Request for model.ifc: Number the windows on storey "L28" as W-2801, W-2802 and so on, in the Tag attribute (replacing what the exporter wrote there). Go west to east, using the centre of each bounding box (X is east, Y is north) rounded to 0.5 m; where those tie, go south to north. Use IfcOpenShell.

First a look at what the model holds.

```python
import ifcopenshell
import ifcopenshell.util.element
import ifcopenshell.util.placement

model = ifcopenshell.open("model.ifc")
print(model.schema)
storey = next(s for s in model.by_type("IfcBuildingStorey") if s.Name == "L28")
windows = [e for e in ifcopenshell.util.element.get_decomposition(storey) if e.is_a("IfcWindow")]
for e in sorted(windows, key=lambda e: e.id()):
    origin = ifcopenshell.util.placement.get_local_placement(e.ObjectPlacement)[:3, 3]
    print(e.id(), e.Tag, e.Name, origin.round(2) + 0.0, sep=" | ")
```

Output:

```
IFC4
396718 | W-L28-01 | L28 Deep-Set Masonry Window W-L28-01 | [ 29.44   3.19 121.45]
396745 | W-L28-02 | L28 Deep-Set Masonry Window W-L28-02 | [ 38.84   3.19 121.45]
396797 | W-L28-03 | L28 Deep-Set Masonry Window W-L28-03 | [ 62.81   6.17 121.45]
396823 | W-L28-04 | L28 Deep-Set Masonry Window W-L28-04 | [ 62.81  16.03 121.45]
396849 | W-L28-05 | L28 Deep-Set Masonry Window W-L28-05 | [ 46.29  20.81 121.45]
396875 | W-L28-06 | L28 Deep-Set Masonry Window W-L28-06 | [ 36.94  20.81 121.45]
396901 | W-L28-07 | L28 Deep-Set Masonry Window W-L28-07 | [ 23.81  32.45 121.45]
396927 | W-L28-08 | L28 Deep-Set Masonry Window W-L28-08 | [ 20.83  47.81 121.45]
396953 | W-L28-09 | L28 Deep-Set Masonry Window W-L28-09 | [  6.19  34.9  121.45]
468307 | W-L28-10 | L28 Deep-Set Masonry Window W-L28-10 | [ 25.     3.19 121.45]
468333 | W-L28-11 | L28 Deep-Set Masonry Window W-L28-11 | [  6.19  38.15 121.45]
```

```python
import ifcopenshell
import ifcopenshell.geom
import ifcopenshell.util.element
import ifcopenshell.util.shape

model = ifcopenshell.open("model.ifc")
settings = ifcopenshell.geom.settings()
settings.set("use-world-coords", True)


def centre(element):
    shape = ifcopenshell.geom.create_shape(settings, element)
    return ifcopenshell.util.shape.get_bbox_centroid(shape.geometry)


storey = next(s for s in model.by_type("IfcBuildingStorey") if s.Name == "L28")
windows = [e for e in ifcopenshell.util.element.get_decomposition(storey) if e.is_a("IfcWindow")]

# Insertion points can sit at a corner or the storey origin, so sort by the geometry (in metres).
centres = {e: centre(e) for e in windows}
windows.sort(key=lambda e: (round(centres[e][0] / 0.5), centres[e][1]))

for i, e in enumerate(windows, start=1):
    number = f"W-28{i:02d}"
    e.Tag = number
    print(e.id(), number)

model.write("model_updated.ifc")
```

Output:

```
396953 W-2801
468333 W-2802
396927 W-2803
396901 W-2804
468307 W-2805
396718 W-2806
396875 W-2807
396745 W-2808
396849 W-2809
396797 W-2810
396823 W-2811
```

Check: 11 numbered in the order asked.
